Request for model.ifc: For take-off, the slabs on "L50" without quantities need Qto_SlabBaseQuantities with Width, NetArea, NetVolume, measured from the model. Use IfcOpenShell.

First a look at what the model holds.

```python
import ifcopenshell
import ifcopenshell.util.element
import ifcopenshell.util.unit

model = ifcopenshell.open("model.ifc")
print(model.schema)
for unit_type in ("LENGTHUNIT", "AREAUNIT", "VOLUMEUNIT"):
    print(unit_type, ifcopenshell.util.unit.calculate_unit_scale(model, unit_type))
storey = next(s for s in model.by_type("IfcBuildingStorey") if s.Name == "L50")
slabs = [e for e in ifcopenshell.util.element.get_decomposition(storey) if e.is_a("IfcSlab")]
for e in sorted(slabs, key=lambda e: e.id()):
    print(e.id(), e.is_a(), e.Name, list(ifcopenshell.util.element.get_psets(e, qtos_only=True)), sep=" | ")
```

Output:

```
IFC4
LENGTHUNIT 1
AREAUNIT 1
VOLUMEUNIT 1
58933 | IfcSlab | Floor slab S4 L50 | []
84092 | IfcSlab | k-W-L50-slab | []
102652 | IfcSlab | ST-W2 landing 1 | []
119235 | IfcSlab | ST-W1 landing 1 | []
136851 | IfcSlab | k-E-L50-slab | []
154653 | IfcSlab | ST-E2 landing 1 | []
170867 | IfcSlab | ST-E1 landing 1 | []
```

```python
import ifcopenshell
import ifcopenshell.api.pset
import ifcopenshell.geom
import ifcopenshell.util.element
import ifcopenshell.util.shape
import ifcopenshell.util.unit

model = ifcopenshell.open("model.ifc")
unit_scale = ifcopenshell.util.unit.calculate_unit_scale(model)
area_scale = ifcopenshell.util.unit.calculate_unit_scale(model, "AREAUNIT")
volume_scale = ifcopenshell.util.unit.calculate_unit_scale(model, "VOLUMEUNIT")
settings = ifcopenshell.geom.settings()

storey = next(s for s in model.by_type("IfcBuildingStorey") if s.Name == "L50")
slabs = [e for e in ifcopenshell.util.element.get_decomposition(storey) if e.is_a("IfcSlab")]

for e in sorted(slabs, key=lambda e: e.id()):
    if ifcopenshell.util.element.get_psets(e, qtos_only=True, should_inherit=False):
        continue
    # Geometry comes back in metres, in the element's own axes.
    shape = ifcopenshell.geom.create_shape(settings, e)
    values = {
        "Width": ifcopenshell.util.shape.get_z(shape.geometry) / unit_scale,
        "NetArea": ifcopenshell.util.shape.get_footprint_area(shape.geometry) / area_scale,
        "NetVolume": ifcopenshell.util.shape.get_volume(shape.geometry) / volume_scale,
    }
    qto = ifcopenshell.api.pset.add_qto(model, product=e, name="Qto_SlabBaseQuantities")
    ifcopenshell.api.pset.edit_qto(model, qto=qto, properties=values)
    print(e.id(), {k: round(v, 3) for k, v in values.items()})

model.write("model_v2.ifc")
```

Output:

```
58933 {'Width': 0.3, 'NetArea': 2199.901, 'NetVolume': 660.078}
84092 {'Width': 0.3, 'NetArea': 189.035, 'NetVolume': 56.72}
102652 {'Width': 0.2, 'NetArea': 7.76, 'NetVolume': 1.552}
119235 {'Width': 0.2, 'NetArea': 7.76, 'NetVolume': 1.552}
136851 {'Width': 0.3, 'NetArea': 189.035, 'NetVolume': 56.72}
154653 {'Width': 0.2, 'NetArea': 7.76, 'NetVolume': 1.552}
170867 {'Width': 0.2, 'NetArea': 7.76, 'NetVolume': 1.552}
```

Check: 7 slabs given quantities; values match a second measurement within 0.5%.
